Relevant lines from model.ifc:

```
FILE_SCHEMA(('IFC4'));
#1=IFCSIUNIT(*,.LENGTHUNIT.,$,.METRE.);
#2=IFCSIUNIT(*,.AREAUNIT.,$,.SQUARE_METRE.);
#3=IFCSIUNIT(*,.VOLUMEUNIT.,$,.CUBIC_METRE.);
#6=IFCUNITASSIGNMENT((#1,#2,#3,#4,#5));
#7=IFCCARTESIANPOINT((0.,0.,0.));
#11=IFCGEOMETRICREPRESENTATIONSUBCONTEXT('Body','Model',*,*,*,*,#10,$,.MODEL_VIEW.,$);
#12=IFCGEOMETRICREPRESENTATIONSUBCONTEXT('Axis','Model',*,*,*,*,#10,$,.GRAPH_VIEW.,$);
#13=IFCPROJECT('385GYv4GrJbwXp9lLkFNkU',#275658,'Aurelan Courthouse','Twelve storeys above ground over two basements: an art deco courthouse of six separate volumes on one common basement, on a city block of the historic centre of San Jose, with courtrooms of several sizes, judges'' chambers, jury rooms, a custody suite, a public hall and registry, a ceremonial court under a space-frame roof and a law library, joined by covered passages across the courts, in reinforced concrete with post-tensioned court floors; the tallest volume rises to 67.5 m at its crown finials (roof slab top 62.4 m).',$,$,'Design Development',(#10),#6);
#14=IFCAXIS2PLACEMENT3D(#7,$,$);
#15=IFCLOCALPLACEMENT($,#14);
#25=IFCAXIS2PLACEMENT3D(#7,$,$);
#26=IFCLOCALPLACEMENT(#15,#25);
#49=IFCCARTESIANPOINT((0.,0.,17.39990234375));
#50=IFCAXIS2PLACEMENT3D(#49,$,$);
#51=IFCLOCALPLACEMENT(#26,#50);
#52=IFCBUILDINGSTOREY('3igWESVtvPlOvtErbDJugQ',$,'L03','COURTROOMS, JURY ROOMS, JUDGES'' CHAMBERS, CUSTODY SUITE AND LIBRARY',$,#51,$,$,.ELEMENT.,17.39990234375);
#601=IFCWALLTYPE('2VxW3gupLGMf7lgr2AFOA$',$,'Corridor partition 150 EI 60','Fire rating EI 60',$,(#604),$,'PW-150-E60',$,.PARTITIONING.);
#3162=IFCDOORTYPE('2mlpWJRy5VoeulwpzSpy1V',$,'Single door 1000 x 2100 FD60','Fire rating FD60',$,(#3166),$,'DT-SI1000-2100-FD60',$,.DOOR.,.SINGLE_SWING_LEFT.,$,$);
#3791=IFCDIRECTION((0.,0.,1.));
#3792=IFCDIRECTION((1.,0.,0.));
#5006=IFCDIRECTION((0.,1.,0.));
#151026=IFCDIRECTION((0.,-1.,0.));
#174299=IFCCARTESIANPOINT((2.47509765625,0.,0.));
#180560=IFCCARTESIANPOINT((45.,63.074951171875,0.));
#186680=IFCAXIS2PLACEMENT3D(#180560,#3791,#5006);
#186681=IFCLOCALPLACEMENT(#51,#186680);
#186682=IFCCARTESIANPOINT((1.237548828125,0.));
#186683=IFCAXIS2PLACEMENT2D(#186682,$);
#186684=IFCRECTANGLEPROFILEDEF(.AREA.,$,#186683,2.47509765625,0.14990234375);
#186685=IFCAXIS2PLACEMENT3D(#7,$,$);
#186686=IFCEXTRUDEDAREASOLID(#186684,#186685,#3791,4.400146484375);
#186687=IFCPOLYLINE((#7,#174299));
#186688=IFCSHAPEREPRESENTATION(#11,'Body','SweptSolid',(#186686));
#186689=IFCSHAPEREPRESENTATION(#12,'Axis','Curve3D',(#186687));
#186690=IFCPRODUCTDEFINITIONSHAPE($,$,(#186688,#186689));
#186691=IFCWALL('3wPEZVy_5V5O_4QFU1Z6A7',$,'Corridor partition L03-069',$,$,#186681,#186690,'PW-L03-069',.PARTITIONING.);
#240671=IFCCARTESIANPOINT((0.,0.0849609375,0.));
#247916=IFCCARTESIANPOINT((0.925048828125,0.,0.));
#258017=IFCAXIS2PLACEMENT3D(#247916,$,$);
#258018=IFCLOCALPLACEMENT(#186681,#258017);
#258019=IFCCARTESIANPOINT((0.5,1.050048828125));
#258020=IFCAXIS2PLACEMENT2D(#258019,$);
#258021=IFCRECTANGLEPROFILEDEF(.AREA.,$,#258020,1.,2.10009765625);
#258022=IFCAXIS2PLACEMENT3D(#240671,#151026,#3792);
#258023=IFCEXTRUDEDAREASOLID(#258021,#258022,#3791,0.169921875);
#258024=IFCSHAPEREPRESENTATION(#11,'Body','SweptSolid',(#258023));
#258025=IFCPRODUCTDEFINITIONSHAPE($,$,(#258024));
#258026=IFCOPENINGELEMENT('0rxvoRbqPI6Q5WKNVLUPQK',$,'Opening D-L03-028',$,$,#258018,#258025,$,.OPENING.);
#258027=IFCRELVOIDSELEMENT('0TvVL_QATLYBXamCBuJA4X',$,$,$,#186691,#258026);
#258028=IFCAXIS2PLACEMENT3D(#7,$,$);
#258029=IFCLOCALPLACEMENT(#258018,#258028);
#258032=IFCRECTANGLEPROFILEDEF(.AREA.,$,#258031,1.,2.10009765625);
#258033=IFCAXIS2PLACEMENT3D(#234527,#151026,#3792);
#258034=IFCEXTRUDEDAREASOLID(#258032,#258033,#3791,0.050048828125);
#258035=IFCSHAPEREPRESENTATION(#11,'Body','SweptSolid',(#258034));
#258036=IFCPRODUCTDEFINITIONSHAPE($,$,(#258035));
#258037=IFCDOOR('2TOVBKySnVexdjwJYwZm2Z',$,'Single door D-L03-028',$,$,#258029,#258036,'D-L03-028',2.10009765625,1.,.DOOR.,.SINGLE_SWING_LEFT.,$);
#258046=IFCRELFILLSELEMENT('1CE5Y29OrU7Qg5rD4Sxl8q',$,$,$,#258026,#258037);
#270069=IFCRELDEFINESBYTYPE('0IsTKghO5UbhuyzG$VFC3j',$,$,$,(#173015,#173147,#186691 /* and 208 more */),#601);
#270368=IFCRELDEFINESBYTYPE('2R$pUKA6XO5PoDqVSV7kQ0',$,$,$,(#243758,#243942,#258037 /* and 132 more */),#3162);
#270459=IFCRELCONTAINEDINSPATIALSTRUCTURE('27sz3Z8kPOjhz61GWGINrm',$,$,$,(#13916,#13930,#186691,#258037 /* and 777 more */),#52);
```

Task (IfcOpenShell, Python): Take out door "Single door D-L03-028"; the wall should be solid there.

```python
import ifcopenshell
import ifcopenshell.api.feature
import ifcopenshell.api.root
import ifcopenshell.geom
import ifcopenshell.util.shape

model = ifcopenshell.open("model.ifc")
settings = ifcopenshell.geom.settings()


def volume(element):
    """Net volume in cubic metres, openings subtracted."""
    shape = ifcopenshell.geom.create_shape(settings, element)
    return ifcopenshell.util.shape.get_volume(shape.geometry)


door = model.by_guid("2TOVBKySnVexdjwJYwZm2Z")
opening = door.FillsVoids[0].RelatingOpeningElement
wall = opening.VoidsElements[0].RelatingBuildingElement
before = volume(wall)

ifcopenshell.api.root.remove_product(model, product=door)
ifcopenshell.api.feature.remove_feature(model, feature=opening)

after = volume(wall)

print(f"wall volume {before:.3f} -> {after:.3f} m3")

model.write("model_v2.ifc")
```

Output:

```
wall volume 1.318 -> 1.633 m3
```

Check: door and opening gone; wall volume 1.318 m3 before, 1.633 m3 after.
